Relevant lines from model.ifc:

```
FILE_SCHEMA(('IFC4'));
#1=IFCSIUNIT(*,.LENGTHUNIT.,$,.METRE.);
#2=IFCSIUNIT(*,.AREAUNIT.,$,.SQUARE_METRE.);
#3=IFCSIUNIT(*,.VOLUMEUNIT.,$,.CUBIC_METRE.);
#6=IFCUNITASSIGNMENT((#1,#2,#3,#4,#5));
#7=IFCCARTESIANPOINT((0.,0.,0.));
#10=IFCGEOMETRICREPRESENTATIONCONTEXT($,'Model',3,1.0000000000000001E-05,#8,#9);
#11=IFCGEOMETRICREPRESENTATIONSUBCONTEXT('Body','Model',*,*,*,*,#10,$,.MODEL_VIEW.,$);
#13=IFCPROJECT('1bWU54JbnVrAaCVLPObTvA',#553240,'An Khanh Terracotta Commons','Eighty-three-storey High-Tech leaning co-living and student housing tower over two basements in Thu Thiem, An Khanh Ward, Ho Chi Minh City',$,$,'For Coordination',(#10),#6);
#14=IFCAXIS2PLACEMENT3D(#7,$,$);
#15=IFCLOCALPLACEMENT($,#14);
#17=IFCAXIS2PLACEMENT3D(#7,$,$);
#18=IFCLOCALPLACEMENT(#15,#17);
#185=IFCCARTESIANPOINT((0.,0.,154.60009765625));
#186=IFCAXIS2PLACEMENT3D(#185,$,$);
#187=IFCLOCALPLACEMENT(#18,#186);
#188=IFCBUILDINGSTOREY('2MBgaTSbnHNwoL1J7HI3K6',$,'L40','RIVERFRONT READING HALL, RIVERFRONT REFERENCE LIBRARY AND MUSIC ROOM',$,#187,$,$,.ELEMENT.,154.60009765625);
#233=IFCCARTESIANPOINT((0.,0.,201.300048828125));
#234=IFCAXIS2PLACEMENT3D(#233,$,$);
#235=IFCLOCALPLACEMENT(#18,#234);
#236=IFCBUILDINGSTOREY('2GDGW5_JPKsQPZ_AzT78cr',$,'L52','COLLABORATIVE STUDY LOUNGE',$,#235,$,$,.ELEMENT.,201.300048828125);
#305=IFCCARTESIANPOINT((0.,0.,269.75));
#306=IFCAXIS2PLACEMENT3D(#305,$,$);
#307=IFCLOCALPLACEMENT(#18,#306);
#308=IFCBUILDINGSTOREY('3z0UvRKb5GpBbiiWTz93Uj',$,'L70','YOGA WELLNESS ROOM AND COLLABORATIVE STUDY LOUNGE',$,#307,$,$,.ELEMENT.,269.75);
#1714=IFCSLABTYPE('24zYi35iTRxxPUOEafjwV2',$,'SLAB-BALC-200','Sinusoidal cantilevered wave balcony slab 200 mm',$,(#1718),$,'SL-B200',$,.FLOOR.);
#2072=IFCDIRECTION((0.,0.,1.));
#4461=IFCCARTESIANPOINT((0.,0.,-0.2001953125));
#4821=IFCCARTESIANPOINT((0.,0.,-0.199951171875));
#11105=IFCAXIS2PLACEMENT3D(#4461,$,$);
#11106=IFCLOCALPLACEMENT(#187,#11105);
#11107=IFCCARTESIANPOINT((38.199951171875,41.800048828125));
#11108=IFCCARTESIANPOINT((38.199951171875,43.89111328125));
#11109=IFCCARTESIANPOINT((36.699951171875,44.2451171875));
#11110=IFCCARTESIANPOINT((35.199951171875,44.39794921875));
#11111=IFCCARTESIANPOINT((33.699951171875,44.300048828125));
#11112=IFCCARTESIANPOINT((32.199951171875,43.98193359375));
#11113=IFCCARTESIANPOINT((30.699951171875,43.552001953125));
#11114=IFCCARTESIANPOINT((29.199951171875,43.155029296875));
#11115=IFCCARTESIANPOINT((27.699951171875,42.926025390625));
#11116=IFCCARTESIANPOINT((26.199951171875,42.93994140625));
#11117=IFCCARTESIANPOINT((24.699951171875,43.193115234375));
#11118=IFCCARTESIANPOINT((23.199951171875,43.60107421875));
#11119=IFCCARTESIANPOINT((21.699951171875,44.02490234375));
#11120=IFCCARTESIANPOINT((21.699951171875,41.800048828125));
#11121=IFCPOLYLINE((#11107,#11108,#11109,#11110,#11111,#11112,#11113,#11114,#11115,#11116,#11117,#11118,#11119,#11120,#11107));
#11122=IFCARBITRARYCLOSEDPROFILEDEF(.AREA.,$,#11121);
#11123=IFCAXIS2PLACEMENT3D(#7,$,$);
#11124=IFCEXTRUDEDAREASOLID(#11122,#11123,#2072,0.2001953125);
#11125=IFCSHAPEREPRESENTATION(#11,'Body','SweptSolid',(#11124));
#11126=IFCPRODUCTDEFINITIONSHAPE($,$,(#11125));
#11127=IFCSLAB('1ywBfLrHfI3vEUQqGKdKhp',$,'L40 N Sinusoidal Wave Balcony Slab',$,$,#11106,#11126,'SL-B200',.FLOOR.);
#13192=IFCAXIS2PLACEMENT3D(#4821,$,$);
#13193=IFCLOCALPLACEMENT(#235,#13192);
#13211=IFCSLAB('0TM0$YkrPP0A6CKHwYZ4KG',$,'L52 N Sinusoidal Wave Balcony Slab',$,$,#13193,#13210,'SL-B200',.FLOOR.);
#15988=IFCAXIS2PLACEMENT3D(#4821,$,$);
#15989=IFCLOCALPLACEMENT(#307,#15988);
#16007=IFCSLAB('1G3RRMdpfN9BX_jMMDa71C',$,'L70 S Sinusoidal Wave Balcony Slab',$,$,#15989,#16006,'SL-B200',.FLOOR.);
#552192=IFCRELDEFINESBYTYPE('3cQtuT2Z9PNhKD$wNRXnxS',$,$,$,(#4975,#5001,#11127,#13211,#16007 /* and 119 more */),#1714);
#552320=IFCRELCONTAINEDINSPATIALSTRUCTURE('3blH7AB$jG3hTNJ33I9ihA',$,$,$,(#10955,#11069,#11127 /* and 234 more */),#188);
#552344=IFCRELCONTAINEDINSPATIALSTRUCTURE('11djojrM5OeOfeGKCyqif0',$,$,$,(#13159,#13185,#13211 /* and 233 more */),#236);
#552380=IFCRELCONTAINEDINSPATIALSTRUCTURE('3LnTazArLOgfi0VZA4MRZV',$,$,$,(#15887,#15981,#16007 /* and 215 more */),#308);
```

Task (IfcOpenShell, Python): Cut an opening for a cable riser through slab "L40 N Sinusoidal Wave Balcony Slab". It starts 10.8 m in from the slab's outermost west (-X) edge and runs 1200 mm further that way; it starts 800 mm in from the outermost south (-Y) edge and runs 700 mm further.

```python
import numpy as np
import ifcopenshell
import ifcopenshell.api.feature
import ifcopenshell.api.geometry
import ifcopenshell.api.root
import ifcopenshell.geom
import ifcopenshell.util.placement
import ifcopenshell.util.representation
import ifcopenshell.util.shape
import ifcopenshell.util.unit

model = ifcopenshell.open("model.ifc")
unit_scale = ifcopenshell.util.unit.calculate_unit_scale(model)
settings = ifcopenshell.geom.settings()


def volume(element):
    """Net volume in cubic metres, openings subtracted."""
    shape = ifcopenshell.geom.create_shape(settings, element)
    return ifcopenshell.util.shape.get_volume(shape.geometry)


slab = model.by_guid("1ywBfLrHfI3vEUQqGKdKhp")
before = volume(slab)

# Extent in the slab's own axes, in metres. The edges named are its -X and -Y sides.
slab_shape = ifcopenshell.geom.create_shape(settings, slab)
vertices = ifcopenshell.util.shape.get_vertices(slab_shape.geometry)
x_min, y_min, bottom = vertices.min(axis=0)
top = vertices[:, 2].max()

opening = ifcopenshell.api.root.create_entity(model, ifc_class="IfcOpeningElement", name="Cable riser opening", predefined_type="OPENING")
context = ifcopenshell.util.representation.get_context(model, "Model", "Body", "MODEL_VIEW")
width, depth = 1.2, 0.7
outline = [(0.0, 0.0), (width, 0.0), (width, depth), (0.0, depth), (0.0, 0.0)]
# Overshoot both faces by 50 mm so the cut is clean.
shape = ifcopenshell.api.geometry.add_slab_representation(
    model, context=context, depth=top - bottom + 0.1, polyline=outline
)
ifcopenshell.api.geometry.assign_representation(model, product=opening, representation=shape)

matrix = ifcopenshell.util.placement.get_local_placement(slab.ObjectPlacement)
matrix[:, 3] = matrix @ np.append(np.array([x_min + 10.8, y_min + 0.8, bottom - 0.05]) / unit_scale, 1.0)
ifcopenshell.api.geometry.edit_object_placement(model, product=opening, matrix=matrix, is_si=False)
ifcopenshell.api.feature.add_feature(model, feature=opening, element=slab)

after = volume(slab)

print(f"slab volume {before:.3f} -> {after:.3f} m3")

model.write("model_v2.ifc")
```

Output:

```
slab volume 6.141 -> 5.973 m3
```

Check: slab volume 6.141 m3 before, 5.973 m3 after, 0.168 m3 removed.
